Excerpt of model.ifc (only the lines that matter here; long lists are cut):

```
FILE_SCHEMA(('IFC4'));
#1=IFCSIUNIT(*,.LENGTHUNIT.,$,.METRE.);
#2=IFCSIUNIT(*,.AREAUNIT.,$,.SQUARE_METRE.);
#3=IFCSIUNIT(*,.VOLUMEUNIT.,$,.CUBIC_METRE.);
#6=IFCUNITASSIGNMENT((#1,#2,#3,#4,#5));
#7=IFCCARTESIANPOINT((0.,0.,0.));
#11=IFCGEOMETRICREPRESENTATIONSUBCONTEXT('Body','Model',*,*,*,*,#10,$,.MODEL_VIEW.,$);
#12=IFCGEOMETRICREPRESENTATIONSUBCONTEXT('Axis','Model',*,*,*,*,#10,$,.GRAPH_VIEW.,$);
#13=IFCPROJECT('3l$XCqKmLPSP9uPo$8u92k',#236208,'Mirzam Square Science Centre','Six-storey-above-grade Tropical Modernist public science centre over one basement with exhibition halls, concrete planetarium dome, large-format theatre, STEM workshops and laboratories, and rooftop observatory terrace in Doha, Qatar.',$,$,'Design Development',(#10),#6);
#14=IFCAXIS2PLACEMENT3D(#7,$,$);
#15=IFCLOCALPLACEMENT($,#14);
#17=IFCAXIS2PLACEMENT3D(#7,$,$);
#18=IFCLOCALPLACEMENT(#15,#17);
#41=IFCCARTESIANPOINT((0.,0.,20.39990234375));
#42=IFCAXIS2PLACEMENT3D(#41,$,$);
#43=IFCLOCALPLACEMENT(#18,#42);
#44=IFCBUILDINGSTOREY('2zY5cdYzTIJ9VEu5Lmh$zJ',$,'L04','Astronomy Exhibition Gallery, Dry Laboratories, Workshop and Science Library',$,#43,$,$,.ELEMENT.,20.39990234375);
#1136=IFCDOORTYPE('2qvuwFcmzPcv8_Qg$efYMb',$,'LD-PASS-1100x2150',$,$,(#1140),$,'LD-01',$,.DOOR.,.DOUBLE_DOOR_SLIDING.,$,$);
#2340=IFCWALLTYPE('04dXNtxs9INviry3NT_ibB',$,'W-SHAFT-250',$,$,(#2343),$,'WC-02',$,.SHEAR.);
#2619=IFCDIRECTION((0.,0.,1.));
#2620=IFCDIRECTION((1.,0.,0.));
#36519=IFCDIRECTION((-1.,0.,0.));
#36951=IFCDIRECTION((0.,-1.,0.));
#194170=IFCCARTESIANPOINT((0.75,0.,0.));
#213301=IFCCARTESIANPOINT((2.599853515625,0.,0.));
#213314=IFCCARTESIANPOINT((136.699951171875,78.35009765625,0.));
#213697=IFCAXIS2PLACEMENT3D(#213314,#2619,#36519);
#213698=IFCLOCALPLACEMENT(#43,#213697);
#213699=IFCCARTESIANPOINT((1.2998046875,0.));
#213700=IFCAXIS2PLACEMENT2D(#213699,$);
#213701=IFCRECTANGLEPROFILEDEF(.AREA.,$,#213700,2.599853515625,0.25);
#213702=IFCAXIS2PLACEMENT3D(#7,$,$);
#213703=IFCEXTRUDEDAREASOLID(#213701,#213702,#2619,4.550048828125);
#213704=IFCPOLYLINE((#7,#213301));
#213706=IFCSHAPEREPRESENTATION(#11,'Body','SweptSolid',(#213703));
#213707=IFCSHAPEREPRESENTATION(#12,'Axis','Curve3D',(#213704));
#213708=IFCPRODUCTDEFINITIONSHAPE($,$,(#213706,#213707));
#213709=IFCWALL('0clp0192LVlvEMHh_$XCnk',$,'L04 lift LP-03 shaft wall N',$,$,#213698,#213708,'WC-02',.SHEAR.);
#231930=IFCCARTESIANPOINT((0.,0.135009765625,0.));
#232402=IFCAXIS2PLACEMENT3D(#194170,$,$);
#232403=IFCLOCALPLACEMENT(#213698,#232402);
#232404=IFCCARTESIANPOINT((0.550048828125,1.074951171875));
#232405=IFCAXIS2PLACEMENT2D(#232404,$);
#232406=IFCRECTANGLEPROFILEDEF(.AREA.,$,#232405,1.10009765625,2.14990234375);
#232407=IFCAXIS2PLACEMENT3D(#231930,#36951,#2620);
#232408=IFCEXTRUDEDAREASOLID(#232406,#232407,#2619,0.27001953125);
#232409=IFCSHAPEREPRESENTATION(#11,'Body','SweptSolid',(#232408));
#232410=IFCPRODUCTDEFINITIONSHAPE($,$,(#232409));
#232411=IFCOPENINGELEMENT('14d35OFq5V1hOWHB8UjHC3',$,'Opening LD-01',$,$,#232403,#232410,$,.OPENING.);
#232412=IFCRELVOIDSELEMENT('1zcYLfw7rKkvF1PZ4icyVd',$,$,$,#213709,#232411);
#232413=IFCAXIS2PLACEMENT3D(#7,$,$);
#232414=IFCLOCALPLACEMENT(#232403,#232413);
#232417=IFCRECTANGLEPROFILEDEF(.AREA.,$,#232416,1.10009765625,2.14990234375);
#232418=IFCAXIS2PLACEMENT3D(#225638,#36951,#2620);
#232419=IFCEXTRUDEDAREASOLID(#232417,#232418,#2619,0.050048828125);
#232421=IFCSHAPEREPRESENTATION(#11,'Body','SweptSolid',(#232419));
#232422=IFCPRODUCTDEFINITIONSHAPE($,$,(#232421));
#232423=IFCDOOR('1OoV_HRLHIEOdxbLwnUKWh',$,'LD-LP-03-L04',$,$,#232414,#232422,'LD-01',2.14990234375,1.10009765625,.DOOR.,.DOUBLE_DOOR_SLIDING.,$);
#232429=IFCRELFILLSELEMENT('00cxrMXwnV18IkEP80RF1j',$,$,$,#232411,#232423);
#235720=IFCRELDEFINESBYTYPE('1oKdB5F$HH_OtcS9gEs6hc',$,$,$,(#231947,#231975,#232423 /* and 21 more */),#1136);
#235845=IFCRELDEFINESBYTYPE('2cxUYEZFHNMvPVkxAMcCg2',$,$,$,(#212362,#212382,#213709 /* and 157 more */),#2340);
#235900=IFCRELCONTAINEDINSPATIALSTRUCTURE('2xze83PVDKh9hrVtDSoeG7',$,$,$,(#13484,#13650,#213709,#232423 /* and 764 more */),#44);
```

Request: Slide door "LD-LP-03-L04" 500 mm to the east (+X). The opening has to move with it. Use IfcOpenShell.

```python
import ifcopenshell
import ifcopenshell.api.geometry
import ifcopenshell.util.placement
import ifcopenshell.util.unit

model = ifcopenshell.open("model.ifc")
unit_scale = ifcopenshell.util.unit.calculate_unit_scale(model)

door = model.by_id(232423)
opening = door.FillsVoids[0].RelatingOpeningElement
wall = opening.VoidsElements[0].RelatingBuildingElement

wall_matrix = ifcopenshell.util.placement.get_local_placement(wall.ObjectPlacement)
shift = wall_matrix[:3, 0] * -0.5 / unit_scale
before = ifcopenshell.util.placement.get_local_placement(door.ObjectPlacement)[:3, 3].copy()

# The door is placed relative to its opening, so it follows when the opening moves.
matrix = ifcopenshell.util.placement.get_local_placement(opening.ObjectPlacement)
matrix[:3, 3] += shift
ifcopenshell.api.geometry.edit_object_placement(
    model, product=opening, matrix=matrix, is_si=False, should_transform_children=True
)

after = ifcopenshell.util.placement.get_local_placement(door.ObjectPlacement)[:3, 3]
print("door moved by", (after - before).round(3) + 0.0)

model.write("model-out.ifc")
```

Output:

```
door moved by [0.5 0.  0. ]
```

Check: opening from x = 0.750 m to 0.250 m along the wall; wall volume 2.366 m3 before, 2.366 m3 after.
